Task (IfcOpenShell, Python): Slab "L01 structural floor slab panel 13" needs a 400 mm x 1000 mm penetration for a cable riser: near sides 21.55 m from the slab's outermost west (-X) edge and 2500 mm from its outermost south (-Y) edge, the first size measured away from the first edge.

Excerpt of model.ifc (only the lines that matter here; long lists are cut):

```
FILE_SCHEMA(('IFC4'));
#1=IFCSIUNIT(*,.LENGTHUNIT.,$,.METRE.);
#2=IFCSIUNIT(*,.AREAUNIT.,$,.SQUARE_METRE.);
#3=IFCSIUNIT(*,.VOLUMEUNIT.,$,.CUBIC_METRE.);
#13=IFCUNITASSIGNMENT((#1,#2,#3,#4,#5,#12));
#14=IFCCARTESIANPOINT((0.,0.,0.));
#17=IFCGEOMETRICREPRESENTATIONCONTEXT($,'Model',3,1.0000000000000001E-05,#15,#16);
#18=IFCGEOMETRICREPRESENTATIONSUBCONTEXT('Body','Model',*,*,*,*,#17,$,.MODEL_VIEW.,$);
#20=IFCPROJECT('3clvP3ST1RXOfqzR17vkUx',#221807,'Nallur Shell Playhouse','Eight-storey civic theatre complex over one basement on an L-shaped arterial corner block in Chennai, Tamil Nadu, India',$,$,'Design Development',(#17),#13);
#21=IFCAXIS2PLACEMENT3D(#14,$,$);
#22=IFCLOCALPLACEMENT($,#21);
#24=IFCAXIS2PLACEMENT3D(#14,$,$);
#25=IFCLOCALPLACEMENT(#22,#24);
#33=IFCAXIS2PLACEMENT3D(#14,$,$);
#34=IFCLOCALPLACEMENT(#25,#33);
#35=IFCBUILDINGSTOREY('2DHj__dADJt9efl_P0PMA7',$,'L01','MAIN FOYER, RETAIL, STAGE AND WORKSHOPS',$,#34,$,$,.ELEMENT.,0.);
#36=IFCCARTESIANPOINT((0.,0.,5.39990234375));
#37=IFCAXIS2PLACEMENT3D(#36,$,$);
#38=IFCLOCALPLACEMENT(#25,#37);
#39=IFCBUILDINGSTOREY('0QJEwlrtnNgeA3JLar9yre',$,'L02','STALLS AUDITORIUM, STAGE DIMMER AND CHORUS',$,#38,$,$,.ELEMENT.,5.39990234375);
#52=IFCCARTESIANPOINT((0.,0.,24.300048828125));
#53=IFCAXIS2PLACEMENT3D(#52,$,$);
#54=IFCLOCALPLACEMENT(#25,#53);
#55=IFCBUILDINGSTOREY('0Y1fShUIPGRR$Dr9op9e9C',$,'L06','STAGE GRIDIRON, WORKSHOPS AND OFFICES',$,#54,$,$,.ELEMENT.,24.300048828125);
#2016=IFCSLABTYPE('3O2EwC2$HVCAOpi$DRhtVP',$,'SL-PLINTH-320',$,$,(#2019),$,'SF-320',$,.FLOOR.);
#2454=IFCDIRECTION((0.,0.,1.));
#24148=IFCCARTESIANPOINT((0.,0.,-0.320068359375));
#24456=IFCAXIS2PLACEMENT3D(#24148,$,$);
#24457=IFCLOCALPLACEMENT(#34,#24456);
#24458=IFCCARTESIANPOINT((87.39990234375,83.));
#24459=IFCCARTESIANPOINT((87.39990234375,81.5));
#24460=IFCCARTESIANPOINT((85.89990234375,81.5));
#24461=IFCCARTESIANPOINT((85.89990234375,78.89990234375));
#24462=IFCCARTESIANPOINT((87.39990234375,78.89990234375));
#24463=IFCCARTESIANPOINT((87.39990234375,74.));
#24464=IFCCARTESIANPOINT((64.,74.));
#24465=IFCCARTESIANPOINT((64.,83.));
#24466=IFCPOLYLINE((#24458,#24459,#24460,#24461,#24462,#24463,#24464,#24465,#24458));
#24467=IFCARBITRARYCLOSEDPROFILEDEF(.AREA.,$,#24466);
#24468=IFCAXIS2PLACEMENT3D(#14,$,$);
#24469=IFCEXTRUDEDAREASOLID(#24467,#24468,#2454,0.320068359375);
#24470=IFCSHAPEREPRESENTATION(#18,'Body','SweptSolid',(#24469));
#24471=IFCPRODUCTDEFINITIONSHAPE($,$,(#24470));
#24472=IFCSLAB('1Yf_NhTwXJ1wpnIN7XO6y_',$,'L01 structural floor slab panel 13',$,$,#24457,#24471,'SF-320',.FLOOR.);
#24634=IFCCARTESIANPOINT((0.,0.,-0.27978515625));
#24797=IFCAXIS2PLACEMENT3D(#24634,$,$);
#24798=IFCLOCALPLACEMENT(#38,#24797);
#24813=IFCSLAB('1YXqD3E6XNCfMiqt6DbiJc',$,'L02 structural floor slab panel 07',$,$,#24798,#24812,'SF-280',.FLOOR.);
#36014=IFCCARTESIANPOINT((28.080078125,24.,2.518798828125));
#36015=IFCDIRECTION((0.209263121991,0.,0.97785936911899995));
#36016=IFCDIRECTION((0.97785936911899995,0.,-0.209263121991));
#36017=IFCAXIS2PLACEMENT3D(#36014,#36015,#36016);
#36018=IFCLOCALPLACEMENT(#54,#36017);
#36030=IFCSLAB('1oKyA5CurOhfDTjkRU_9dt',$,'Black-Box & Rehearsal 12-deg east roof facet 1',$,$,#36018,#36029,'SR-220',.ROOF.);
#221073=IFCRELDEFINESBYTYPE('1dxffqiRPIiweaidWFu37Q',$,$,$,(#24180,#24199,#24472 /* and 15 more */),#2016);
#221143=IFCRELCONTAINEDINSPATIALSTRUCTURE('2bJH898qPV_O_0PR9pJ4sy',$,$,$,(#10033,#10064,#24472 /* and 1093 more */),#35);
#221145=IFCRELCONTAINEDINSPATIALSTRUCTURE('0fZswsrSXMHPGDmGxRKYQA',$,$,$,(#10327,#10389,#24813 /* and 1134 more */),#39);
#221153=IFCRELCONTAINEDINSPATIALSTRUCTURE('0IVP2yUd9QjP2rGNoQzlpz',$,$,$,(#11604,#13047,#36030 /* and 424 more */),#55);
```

```python
import numpy as np
import ifcopenshell
import ifcopenshell.api.feature
import ifcopenshell.api.geometry
import ifcopenshell.api.root
import ifcopenshell.geom
import ifcopenshell.util.placement
import ifcopenshell.util.representation
import ifcopenshell.util.shape
import ifcopenshell.util.unit

model = ifcopenshell.open("model.ifc")
unit_scale = ifcopenshell.util.unit.calculate_unit_scale(model)
settings = ifcopenshell.geom.settings()


def volume(element):
    """Net volume in cubic metres, openings subtracted."""
    shape = ifcopenshell.geom.create_shape(settings, element)
    return ifcopenshell.util.shape.get_volume(shape.geometry)


slab = model.by_guid("1Yf_NhTwXJ1wpnIN7XO6y_")
before = volume(slab)

# Extent in the slab's own axes, in metres. The edges named are its -X and -Y sides.
slab_shape = ifcopenshell.geom.create_shape(settings, slab)
vertices = ifcopenshell.util.shape.get_vertices(slab_shape.geometry)
x_min, y_min, bottom = vertices.min(axis=0)
top = vertices[:, 2].max()

opening = ifcopenshell.api.root.create_entity(model, ifc_class="IfcOpeningElement", name="Cable riser opening", predefined_type="OPENING")
context = ifcopenshell.util.representation.get_context(model, "Model", "Body", "MODEL_VIEW")
width, depth = 0.4, 1
outline = [(0.0, 0.0), (width, 0.0), (width, depth), (0.0, depth), (0.0, 0.0)]
# Overshoot both faces by 50 mm so the cut is clean.
shape = ifcopenshell.api.geometry.add_slab_representation(
    model, context=context, depth=top - bottom + 0.1, polyline=outline
)
ifcopenshell.api.geometry.assign_representation(model, product=opening, representation=shape)

matrix = ifcopenshell.util.placement.get_local_placement(slab.ObjectPlacement)
matrix[:, 3] = matrix @ np.append(np.array([x_min + 21.55, y_min + 2.5, bottom - 0.05]) / unit_scale, 1.0)
ifcopenshell.api.geometry.edit_object_placement(model, product=opening, matrix=matrix, is_si=False)
ifcopenshell.api.feature.add_feature(model, feature=opening, element=slab)

after = volume(slab)

print(f"slab volume {before:.3f} -> {after:.3f} m3")

model.write("model_rev.ifc")
```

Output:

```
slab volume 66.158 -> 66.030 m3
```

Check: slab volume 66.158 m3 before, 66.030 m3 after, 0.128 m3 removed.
